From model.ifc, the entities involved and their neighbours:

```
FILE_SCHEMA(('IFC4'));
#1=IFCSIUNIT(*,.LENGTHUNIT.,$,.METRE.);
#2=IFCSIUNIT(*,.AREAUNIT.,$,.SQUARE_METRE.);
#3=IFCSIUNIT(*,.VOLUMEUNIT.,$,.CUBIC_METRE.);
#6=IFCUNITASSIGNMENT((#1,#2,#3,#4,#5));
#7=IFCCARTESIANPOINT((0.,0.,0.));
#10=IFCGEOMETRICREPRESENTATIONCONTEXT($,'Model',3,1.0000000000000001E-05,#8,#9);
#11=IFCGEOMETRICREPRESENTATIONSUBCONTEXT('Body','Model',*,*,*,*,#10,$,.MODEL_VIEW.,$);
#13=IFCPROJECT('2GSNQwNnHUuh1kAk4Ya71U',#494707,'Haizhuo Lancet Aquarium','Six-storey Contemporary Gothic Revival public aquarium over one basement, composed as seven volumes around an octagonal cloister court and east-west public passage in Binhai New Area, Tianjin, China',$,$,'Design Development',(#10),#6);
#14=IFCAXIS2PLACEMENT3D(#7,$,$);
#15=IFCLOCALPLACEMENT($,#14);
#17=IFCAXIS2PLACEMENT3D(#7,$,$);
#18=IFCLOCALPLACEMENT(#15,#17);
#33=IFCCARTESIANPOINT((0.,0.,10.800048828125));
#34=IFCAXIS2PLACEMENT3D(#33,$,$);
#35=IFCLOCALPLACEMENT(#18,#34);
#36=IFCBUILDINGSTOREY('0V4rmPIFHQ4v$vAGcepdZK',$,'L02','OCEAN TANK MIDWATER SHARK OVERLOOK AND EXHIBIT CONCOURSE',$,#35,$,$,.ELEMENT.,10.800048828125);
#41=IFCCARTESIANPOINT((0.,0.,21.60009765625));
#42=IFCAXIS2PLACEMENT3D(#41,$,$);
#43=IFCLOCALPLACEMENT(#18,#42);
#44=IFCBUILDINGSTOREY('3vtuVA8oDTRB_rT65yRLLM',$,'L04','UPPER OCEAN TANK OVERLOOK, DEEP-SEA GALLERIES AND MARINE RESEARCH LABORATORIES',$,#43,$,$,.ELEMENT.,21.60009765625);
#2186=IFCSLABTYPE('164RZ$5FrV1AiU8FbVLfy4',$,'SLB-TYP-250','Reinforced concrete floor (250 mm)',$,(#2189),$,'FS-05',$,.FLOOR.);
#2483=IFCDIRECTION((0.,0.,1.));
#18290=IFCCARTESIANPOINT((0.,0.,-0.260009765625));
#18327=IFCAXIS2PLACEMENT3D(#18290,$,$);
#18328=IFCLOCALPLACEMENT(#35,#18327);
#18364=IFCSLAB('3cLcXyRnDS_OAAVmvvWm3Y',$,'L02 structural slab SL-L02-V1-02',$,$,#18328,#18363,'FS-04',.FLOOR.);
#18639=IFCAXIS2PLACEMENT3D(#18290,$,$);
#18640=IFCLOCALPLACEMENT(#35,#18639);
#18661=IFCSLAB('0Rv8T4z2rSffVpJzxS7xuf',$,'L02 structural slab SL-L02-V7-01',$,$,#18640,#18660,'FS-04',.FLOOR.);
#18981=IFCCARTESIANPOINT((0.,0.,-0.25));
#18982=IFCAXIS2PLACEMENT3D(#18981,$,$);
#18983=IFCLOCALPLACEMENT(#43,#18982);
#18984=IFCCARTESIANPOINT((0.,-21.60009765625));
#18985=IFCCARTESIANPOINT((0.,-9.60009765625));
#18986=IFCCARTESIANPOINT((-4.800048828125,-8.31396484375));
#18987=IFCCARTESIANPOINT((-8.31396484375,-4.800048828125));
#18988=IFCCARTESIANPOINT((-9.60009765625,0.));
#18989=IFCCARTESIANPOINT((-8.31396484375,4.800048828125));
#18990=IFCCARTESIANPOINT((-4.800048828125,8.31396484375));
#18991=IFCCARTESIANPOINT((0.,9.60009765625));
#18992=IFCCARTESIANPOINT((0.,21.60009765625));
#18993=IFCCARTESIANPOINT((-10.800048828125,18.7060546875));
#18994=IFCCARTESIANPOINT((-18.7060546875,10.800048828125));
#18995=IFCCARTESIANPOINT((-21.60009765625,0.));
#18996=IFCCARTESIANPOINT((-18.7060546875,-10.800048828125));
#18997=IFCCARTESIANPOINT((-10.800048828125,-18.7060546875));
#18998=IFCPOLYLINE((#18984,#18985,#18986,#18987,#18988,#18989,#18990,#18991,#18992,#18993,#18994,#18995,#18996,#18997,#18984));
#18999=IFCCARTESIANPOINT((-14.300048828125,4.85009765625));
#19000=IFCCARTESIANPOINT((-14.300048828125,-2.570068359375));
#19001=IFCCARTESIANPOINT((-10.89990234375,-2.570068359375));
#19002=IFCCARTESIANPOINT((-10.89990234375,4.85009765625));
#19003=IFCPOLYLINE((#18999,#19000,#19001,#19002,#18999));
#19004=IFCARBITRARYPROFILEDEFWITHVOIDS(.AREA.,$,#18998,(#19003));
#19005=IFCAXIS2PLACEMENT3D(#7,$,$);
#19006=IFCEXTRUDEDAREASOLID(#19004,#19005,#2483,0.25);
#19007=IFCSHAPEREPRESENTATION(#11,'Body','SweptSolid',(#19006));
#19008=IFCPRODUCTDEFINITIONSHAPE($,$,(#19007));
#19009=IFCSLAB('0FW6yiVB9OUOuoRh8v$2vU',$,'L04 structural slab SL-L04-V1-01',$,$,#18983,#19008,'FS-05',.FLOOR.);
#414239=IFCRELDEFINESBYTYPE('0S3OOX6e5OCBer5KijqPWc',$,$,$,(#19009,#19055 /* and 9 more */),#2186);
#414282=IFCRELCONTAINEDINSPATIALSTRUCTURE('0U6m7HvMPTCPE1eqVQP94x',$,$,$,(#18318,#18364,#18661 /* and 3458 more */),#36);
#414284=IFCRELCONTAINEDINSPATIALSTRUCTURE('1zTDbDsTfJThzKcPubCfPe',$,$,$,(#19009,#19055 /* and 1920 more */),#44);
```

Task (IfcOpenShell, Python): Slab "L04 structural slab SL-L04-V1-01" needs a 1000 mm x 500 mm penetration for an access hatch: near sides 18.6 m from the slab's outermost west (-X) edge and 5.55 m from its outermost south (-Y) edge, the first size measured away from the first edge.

```python
import numpy as np
import ifcopenshell
import ifcopenshell.api.feature
import ifcopenshell.api.geometry
import ifcopenshell.api.root
import ifcopenshell.geom
import ifcopenshell.util.placement
import ifcopenshell.util.representation
import ifcopenshell.util.shape
import ifcopenshell.util.unit

model = ifcopenshell.open("model.ifc")
unit_scale = ifcopenshell.util.unit.calculate_unit_scale(model)
settings = ifcopenshell.geom.settings()


def volume(element):
    """Net volume in cubic metres, openings subtracted."""
    shape = ifcopenshell.geom.create_shape(settings, element)
    return ifcopenshell.util.shape.get_volume(shape.geometry)


slab = model.by_id(19009)
before = volume(slab)

# Extent in the slab's own axes, in metres. The edges named are its -X and -Y sides.
slab_shape = ifcopenshell.geom.create_shape(settings, slab)
vertices = ifcopenshell.util.shape.get_vertices(slab_shape.geometry)
x_min, y_min, bottom = vertices.min(axis=0)
top = vertices[:, 2].max()

opening = ifcopenshell.api.root.create_entity(model, ifc_class="IfcOpeningElement", name="Access hatch opening", predefined_type="OPENING")
context = ifcopenshell.util.representation.get_context(model, "Model", "Body", "MODEL_VIEW")
width, depth = 1, 0.5
outline = [(0.0, 0.0), (width, 0.0), (width, depth), (0.0, depth), (0.0, 0.0)]
# Overshoot both faces by 50 mm so the cut is clean.
shape = ifcopenshell.api.geometry.add_slab_representation(
    model, context=context, depth=top - bottom + 0.1, polyline=outline
)
ifcopenshell.api.geometry.assign_representation(model, product=opening, representation=shape)

matrix = ifcopenshell.util.placement.get_local_placement(slab.ObjectPlacement)
matrix[:, 3] = matrix @ np.append(np.array([x_min + 18.6, y_min + 5.55, bottom - 0.05]) / unit_scale, 1.0)
ifcopenshell.api.geometry.edit_object_placement(model, product=opening, matrix=matrix, is_si=False)
ifcopenshell.api.feature.add_feature(model, feature=opening, element=slab)

after = volume(slab)

print(f"slab volume {before:.3f} -> {after:.3f} m3")

model.write("model-out.ifc")
```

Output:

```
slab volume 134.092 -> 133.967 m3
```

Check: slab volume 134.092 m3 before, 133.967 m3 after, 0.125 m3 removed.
